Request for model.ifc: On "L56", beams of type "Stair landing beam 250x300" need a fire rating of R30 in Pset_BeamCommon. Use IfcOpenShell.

First a look at what the model holds.

```python
import ifcopenshell
import ifcopenshell.util.element

model = ifcopenshell.open("model.ifc")
print(model.schema)
storey = next(s for s in model.by_type("IfcBuildingStorey") if s.Name == "L56")
beams = [e for e in ifcopenshell.util.element.get_decomposition(storey) if e.is_a("IfcBeam")]
seen = {}
for e in beams:
    element_type = ifcopenshell.util.element.get_type(e)
    key = (element_type.Name if element_type != e and element_type else None, ifcopenshell.util.element.get_pset(e, "Pset_BeamCommon", "FireRating"))
    seen[key] = seen.get(key, 0) + 1
for (name, value), count in sorted(seen.items(), key=str):
    print(count, "x", name, "|", value)
```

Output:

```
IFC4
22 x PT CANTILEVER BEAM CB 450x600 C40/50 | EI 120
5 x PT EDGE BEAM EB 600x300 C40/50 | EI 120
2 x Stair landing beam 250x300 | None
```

```python
import ifcopenshell
import ifcopenshell.api.pset
import ifcopenshell.util.element

model = ifcopenshell.open("model.ifc")

storey = next(s for s in model.by_type("IfcBuildingStorey") if s.Name == "L56")
beams = [e for e in ifcopenshell.util.element.get_decomposition(storey) if e.is_a("IfcBeam")]

count = 0
for e in beams:
    element_type = ifcopenshell.util.element.get_type(e)
    if element_type in (None, e) or element_type.Name != "Stair landing beam 250x300":
        continue
    found = ifcopenshell.util.element.get_pset(e, "Pset_BeamCommon", should_inherit=False)
    if found:
        pset = model.by_id(found["id"])
        if len(ifcopenshell.util.element.get_elements_by_pset(pset)) > 1:
            pset = ifcopenshell.api.pset.unshare_pset(model, products=[e], pset=pset)[0]
    else:
        pset = ifcopenshell.api.pset.add_pset(model, product=e, name="Pset_BeamCommon")
    ifcopenshell.api.pset.edit_pset(model, pset=pset, properties={"FireRating": "R30"})
    count += 1

print(count, "beams updated")

model.write("model-out.ifc")
```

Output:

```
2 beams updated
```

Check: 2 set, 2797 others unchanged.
